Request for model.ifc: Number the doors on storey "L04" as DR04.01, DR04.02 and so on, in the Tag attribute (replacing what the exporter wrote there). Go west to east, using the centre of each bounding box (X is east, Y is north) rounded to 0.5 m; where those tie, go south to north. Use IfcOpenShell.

First a look at what the model holds.

```python
import ifcopenshell
import ifcopenshell.util.element
import ifcopenshell.util.placement

model = ifcopenshell.open("model.ifc")
print(model.schema)
storey = next(s for s in model.by_type("IfcBuildingStorey") if s.Name == "L04")
doors = [e for e in ifcopenshell.util.element.get_decomposition(storey) if e.is_a("IfcDoor")]
for e in sorted(doors, key=lambda e: e.id()):
    origin = ifcopenshell.util.placement.get_local_placement(e.ObjectPlacement)[:3, 3]
    print(e.id(), e.Tag, e.Name, origin.round(2) + 0.0, sep=" | ")
```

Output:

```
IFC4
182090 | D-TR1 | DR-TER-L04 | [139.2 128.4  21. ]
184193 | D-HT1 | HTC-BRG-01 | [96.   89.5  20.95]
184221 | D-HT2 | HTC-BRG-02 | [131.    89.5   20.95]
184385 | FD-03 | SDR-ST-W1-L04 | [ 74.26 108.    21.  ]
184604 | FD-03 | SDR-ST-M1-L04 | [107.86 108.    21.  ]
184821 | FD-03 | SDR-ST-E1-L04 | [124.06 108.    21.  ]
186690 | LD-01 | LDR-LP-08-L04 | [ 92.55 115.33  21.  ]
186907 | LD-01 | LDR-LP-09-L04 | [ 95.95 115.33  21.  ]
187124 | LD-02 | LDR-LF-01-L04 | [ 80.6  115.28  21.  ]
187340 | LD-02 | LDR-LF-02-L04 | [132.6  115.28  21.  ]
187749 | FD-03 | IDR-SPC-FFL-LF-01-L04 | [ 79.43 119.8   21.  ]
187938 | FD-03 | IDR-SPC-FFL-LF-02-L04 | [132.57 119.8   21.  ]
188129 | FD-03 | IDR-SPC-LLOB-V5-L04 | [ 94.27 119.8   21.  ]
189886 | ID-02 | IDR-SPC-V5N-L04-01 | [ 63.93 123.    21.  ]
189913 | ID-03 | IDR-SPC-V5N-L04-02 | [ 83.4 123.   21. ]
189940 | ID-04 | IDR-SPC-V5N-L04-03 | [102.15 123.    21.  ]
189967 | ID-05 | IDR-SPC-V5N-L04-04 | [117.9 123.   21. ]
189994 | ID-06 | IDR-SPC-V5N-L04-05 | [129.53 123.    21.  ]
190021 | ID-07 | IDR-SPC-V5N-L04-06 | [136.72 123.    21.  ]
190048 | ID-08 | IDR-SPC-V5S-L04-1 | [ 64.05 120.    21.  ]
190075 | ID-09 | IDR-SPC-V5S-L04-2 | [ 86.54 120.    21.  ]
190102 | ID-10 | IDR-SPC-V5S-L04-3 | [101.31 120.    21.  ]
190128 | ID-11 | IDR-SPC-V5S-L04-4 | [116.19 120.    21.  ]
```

```python
import ifcopenshell
import ifcopenshell.geom
import ifcopenshell.util.element
import ifcopenshell.util.shape

model = ifcopenshell.open("model.ifc")
settings = ifcopenshell.geom.settings()
settings.set("use-world-coords", True)


def centre(element):
    shape = ifcopenshell.geom.create_shape(settings, element)
    return ifcopenshell.util.shape.get_bbox_centroid(shape.geometry)


storey = next(s for s in model.by_type("IfcBuildingStorey") if s.Name == "L04")
doors = [e for e in ifcopenshell.util.element.get_decomposition(storey) if e.is_a("IfcDoor")]

# Insertion points can sit at a corner or the storey origin, so sort by the geometry (in metres).
centres = {e: centre(e) for e in doors}
doors.sort(key=lambda e: (round(centres[e][0] / 0.5), centres[e][1]))

for i, e in enumerate(doors, start=1):
    number = f"DR04.{i:02d}"
    e.Tag = number
    print(e.id(), number)

model.write("model-out.ifc")
```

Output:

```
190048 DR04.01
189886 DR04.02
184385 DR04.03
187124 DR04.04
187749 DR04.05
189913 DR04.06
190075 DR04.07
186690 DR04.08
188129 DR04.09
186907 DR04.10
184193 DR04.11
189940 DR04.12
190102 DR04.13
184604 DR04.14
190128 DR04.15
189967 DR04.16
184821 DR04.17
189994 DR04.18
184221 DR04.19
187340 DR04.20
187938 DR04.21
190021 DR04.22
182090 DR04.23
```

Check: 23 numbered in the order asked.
